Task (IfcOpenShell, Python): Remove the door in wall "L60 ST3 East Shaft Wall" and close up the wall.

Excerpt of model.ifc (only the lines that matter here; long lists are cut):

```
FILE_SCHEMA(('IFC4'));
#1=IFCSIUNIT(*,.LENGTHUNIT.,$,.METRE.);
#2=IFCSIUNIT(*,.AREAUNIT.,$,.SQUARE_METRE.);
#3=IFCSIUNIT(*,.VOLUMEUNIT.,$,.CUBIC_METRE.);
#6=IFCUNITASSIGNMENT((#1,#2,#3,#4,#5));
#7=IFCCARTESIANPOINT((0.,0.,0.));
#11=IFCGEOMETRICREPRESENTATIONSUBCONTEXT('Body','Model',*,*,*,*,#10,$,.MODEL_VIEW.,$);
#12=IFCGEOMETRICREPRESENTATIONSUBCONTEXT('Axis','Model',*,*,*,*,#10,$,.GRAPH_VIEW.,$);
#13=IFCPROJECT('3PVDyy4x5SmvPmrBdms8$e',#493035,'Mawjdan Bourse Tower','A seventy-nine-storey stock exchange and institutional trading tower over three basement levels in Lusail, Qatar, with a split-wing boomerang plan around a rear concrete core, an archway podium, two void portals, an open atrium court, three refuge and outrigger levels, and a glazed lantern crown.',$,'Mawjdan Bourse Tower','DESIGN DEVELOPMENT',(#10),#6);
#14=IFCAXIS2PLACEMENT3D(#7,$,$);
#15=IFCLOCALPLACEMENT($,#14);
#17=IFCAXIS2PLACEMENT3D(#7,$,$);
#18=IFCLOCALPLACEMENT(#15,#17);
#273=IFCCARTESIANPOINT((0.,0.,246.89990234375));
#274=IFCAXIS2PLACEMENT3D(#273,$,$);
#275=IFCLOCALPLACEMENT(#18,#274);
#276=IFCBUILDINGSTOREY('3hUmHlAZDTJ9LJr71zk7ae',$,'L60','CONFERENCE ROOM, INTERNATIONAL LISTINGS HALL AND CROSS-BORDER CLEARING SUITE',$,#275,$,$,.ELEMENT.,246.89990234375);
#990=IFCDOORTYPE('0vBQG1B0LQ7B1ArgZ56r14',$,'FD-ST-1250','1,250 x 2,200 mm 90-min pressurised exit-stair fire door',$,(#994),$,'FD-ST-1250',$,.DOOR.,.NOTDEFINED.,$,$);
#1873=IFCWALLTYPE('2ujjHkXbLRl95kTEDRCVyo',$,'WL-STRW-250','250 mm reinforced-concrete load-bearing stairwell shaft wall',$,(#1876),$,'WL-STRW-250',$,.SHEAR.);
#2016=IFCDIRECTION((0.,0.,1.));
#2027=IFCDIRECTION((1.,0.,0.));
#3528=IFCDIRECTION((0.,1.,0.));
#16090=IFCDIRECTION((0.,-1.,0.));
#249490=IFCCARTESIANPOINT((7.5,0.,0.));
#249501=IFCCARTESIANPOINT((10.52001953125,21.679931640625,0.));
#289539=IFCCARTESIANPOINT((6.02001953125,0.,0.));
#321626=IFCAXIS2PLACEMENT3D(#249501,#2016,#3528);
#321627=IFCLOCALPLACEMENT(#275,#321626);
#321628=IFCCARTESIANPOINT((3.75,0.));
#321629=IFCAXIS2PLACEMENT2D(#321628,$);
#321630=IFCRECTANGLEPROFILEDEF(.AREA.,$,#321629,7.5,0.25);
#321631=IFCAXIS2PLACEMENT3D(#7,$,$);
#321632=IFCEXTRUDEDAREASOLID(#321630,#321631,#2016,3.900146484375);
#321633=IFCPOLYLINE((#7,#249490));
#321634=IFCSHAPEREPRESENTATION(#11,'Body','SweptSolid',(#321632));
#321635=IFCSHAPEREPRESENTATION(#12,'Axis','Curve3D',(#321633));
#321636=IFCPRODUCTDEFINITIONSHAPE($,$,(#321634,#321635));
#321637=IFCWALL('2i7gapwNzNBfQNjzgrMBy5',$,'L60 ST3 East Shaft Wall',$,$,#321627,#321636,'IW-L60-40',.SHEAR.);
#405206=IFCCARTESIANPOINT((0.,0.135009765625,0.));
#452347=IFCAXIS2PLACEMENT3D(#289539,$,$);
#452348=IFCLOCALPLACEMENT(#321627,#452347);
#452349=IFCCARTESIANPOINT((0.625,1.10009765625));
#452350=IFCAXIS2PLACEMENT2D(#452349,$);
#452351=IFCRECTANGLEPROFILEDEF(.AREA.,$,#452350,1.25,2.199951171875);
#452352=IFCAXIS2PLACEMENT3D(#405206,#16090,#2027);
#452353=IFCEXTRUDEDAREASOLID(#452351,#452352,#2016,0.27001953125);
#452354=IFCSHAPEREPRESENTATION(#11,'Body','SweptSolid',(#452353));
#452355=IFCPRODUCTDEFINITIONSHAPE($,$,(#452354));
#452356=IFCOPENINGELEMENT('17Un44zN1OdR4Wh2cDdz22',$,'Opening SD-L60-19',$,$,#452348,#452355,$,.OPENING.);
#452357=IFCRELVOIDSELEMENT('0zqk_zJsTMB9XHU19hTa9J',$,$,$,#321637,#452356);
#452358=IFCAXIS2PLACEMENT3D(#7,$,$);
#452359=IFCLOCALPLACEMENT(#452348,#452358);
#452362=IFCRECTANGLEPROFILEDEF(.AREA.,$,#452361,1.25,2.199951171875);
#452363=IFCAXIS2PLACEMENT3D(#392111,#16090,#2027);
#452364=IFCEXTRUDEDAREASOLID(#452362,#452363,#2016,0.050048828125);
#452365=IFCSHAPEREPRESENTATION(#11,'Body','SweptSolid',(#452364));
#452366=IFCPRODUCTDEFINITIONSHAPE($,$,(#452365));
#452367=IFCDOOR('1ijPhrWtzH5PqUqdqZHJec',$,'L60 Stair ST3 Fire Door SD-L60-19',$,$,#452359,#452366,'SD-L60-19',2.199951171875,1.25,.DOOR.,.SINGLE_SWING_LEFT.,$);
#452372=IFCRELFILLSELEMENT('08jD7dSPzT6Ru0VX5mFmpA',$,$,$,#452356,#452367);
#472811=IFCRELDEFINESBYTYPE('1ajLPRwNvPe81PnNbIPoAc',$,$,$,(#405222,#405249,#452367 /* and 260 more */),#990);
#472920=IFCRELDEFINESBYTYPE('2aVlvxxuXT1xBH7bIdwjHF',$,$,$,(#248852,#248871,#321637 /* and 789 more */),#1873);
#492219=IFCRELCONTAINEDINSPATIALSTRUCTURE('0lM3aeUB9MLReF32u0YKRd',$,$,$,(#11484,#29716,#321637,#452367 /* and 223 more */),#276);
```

```python
import ifcopenshell
import ifcopenshell.api.feature
import ifcopenshell.api.root
import ifcopenshell.geom
import ifcopenshell.util.shape

model = ifcopenshell.open("model.ifc")
settings = ifcopenshell.geom.settings()


def volume(element):
    """Net volume in cubic metres, openings subtracted."""
    shape = ifcopenshell.geom.create_shape(settings, element)
    return ifcopenshell.util.shape.get_volume(shape.geometry)


door = model.by_guid("1ijPhrWtzH5PqUqdqZHJec")
opening = door.FillsVoids[0].RelatingOpeningElement
wall = opening.VoidsElements[0].RelatingBuildingElement
before = volume(wall)

ifcopenshell.api.root.remove_product(model, product=door)
ifcopenshell.api.feature.remove_feature(model, feature=opening)

after = volume(wall)

print(f"wall volume {before:.3f} -> {after:.3f} m3")

model.write("model-out.ifc")
```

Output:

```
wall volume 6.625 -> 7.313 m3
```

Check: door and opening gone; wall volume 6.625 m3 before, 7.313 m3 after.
